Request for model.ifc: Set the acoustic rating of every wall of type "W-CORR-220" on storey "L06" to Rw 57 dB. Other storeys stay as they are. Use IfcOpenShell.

First a look at what the model holds.

```python
import ifcopenshell
import ifcopenshell.util.element

model = ifcopenshell.open("model.ifc")
print(model.schema)
storey = next(s for s in model.by_type("IfcBuildingStorey") if s.Name == "L06")
walls = [e for e in ifcopenshell.util.element.get_decomposition(storey) if e.is_a("IfcWall")]
seen = {}
for e in walls:
    element_type = ifcopenshell.util.element.get_type(e)
    key = (element_type.Name if element_type != e and element_type else None, ifcopenshell.util.element.get_pset(e, "Pset_WallCommon", "AcousticRating"))
    seen[key] = seen.get(key, 0) + 1
for (name, value), count in sorted(seen.items(), key=str):
    print(count, "x", name, "|", value)
```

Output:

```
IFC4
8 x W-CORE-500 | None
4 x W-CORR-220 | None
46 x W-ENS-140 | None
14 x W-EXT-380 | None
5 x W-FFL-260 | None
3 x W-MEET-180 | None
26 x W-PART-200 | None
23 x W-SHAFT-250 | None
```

```python
import ifcopenshell
import ifcopenshell.api.pset
import ifcopenshell.util.element

model = ifcopenshell.open("model.ifc")

storey = next(s for s in model.by_type("IfcBuildingStorey") if s.Name == "L06")
walls = [e for e in ifcopenshell.util.element.get_decomposition(storey) if e.is_a("IfcWall")]

count = 0
for e in walls:
    element_type = ifcopenshell.util.element.get_type(e)
    if element_type in (None, e) or element_type.Name != "W-CORR-220":
        continue
    # add_pset returns the element's existing set when there is one.
    pset = ifcopenshell.api.pset.add_pset(model, product=e, name="Pset_WallCommon")
    ifcopenshell.api.pset.edit_pset(model, pset=pset, properties={"AcousticRating": "Rw 57 dB"})
    count += 1

print(count, "walls updated")

model.write("model_updated.ifc")
```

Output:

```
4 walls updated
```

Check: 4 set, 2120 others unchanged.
